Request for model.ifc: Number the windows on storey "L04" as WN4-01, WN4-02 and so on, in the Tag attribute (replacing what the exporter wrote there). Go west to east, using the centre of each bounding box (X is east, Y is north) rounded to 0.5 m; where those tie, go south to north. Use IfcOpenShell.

First a look at what the model holds.

```python
import ifcopenshell
import ifcopenshell.util.element
import ifcopenshell.util.placement

model = ifcopenshell.open("model.ifc")
print(model.schema)
storey = next(s for s in model.by_type("IfcBuildingStorey") if s.Name == "L04")
windows = [e for e in ifcopenshell.util.element.get_decomposition(storey) if e.is_a("IfcWindow")]
for e in sorted(windows, key=lambda e: e.id()):
    origin = ifcopenshell.util.placement.get_local_placement(e.ObjectPlacement)[:3, 3]
    print(e.id(), e.Tag, e.Name, origin.round(2) + 0.0, sep=" | ")
```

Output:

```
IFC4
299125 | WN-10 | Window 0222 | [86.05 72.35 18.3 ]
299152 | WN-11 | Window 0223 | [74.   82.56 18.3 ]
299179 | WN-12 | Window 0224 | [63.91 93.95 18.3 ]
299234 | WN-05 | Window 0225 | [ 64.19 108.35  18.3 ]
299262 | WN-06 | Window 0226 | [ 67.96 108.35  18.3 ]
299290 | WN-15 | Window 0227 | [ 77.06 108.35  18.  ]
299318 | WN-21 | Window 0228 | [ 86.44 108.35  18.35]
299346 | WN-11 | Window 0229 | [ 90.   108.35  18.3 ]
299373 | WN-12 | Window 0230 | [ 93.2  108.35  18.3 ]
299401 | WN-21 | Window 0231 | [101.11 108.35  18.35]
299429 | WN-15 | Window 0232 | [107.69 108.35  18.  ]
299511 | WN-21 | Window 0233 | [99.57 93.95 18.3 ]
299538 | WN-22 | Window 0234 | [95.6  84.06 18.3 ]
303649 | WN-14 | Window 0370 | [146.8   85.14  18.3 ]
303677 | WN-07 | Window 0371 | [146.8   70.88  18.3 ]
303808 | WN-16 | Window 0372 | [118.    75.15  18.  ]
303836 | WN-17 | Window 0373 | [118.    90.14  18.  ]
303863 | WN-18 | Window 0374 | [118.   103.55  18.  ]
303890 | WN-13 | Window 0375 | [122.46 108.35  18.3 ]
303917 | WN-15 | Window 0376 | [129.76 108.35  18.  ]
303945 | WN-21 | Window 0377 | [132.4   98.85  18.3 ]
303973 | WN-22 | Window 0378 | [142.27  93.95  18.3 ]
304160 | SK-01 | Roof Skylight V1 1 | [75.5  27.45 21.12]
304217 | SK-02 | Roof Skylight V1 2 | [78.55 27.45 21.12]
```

```python
import ifcopenshell
import ifcopenshell.geom
import ifcopenshell.util.element
import ifcopenshell.util.shape

model = ifcopenshell.open("model.ifc")
settings = ifcopenshell.geom.settings()
settings.set("use-world-coords", True)


def centre(element):
    shape = ifcopenshell.geom.create_shape(settings, element)
    return ifcopenshell.util.shape.get_bbox_centroid(shape.geometry)


storey = next(s for s in model.by_type("IfcBuildingStorey") if s.Name == "L04")
windows = [e for e in ifcopenshell.util.element.get_decomposition(storey) if e.is_a("IfcWindow")]

# Insertion points can sit at a corner or the storey origin, so sort by the geometry (in metres).
centres = {e: centre(e) for e in windows}
windows.sort(key=lambda e: (round(centres[e][0] / 0.5), centres[e][1]))

for i, e in enumerate(windows, start=1):
    number = f"WN4-{i:02d}"
    e.Tag = number
    print(e.id(), number)

model.write("model_v2.ifc")
```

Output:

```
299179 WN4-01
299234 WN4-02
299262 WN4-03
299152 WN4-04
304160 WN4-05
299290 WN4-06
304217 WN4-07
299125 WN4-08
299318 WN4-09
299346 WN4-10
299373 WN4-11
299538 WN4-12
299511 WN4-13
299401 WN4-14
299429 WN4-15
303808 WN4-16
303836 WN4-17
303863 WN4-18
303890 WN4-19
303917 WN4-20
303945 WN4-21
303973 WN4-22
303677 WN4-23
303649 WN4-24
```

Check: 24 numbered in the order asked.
